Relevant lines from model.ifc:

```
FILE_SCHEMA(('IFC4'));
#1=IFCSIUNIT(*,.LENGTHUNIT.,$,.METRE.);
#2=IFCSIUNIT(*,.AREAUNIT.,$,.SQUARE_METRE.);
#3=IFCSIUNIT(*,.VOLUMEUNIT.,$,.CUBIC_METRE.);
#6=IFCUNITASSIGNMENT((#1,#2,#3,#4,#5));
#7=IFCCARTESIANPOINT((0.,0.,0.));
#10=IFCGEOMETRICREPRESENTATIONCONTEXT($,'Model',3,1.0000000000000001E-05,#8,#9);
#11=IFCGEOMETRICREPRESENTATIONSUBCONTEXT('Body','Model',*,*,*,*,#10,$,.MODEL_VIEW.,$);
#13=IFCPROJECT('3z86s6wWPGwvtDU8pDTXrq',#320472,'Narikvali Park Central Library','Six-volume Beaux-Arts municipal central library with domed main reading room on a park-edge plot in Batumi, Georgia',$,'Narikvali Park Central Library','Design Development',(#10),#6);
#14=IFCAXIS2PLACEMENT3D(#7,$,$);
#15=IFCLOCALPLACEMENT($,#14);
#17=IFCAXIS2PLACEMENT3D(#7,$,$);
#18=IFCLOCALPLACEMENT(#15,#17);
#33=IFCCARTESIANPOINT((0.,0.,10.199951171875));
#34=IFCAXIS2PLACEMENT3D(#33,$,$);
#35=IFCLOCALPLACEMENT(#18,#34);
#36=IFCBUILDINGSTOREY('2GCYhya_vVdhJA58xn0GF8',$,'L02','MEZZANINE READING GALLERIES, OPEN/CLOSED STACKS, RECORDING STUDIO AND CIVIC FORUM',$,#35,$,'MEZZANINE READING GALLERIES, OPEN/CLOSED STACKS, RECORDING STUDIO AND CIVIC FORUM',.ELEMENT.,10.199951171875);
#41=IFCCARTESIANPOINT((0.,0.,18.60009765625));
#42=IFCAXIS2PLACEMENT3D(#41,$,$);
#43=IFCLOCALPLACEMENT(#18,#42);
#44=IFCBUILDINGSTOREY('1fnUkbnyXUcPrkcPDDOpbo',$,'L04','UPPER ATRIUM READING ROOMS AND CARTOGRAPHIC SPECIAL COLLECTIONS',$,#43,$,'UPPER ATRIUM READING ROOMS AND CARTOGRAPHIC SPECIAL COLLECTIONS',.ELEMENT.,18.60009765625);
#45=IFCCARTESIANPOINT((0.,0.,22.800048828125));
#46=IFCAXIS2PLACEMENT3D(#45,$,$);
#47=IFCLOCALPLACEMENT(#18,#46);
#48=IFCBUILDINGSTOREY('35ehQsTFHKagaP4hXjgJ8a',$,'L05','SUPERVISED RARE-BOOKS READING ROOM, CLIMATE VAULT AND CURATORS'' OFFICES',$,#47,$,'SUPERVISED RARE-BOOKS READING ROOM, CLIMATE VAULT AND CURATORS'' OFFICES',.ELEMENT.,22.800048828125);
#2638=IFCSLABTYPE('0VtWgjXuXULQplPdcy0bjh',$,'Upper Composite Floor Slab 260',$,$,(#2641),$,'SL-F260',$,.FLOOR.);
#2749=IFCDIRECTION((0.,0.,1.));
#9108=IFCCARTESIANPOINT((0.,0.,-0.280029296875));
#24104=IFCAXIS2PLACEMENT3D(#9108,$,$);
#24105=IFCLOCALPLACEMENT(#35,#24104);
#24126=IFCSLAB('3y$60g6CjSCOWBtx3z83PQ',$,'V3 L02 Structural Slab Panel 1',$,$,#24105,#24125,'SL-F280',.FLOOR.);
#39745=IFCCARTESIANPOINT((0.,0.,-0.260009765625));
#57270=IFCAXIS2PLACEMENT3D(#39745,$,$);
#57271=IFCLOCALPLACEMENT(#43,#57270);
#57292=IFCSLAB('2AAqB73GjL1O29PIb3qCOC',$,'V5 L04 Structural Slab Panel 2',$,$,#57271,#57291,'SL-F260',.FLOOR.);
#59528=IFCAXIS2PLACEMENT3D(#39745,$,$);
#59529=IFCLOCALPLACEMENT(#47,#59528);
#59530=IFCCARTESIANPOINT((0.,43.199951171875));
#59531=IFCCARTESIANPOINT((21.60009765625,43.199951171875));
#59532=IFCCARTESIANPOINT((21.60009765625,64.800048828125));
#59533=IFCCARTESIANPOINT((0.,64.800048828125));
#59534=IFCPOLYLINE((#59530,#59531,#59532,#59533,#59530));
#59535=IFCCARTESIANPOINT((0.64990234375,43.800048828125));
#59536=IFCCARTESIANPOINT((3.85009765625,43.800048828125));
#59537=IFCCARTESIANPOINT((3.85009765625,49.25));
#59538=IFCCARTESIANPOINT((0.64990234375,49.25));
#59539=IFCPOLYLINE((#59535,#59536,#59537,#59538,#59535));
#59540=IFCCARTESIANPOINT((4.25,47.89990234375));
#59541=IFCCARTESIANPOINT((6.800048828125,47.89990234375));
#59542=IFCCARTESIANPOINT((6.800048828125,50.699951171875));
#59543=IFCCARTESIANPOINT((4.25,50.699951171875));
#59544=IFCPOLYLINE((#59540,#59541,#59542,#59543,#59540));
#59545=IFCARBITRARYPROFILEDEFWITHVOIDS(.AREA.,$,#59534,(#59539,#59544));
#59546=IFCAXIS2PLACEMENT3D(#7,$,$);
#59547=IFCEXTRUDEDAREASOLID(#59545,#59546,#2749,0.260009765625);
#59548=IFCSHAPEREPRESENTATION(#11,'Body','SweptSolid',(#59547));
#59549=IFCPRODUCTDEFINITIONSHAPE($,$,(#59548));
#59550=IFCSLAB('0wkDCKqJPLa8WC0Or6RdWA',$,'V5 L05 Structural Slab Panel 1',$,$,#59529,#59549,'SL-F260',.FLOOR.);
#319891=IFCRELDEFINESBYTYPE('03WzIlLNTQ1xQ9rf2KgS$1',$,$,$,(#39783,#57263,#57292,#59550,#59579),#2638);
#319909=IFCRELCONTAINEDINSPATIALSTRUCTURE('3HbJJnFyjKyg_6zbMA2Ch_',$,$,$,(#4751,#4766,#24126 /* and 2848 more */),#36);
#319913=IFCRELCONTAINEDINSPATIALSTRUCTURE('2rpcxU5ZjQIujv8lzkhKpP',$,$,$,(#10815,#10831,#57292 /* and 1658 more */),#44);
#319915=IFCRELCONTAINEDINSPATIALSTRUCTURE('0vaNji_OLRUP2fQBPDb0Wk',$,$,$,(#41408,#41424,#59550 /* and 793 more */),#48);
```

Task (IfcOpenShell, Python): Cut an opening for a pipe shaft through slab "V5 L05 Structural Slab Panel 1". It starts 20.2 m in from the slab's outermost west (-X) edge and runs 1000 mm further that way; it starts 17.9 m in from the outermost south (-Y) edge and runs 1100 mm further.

```python
import numpy as np
import ifcopenshell
import ifcopenshell.api.feature
import ifcopenshell.api.geometry
import ifcopenshell.api.root
import ifcopenshell.geom
import ifcopenshell.util.placement
import ifcopenshell.util.representation
import ifcopenshell.util.shape
import ifcopenshell.util.unit

model = ifcopenshell.open("model.ifc")
unit_scale = ifcopenshell.util.unit.calculate_unit_scale(model)
settings = ifcopenshell.geom.settings()


def volume(element):
    """Net volume in cubic metres, openings subtracted."""
    shape = ifcopenshell.geom.create_shape(settings, element)
    return ifcopenshell.util.shape.get_volume(shape.geometry)


slab = model.by_guid("0wkDCKqJPLa8WC0Or6RdWA")
before = volume(slab)

# Extent in the slab's own axes, in metres. The edges named are its -X and -Y sides.
slab_shape = ifcopenshell.geom.create_shape(settings, slab)
vertices = ifcopenshell.util.shape.get_vertices(slab_shape.geometry)
x_min, y_min, bottom = vertices.min(axis=0)
top = vertices[:, 2].max()

opening = ifcopenshell.api.root.create_entity(model, ifc_class="IfcOpeningElement", name="Pipe shaft opening", predefined_type="OPENING")
context = ifcopenshell.util.representation.get_context(model, "Model", "Body", "MODEL_VIEW")
width, depth = 1, 1.1
outline = [(0.0, 0.0), (width, 0.0), (width, depth), (0.0, depth), (0.0, 0.0)]
# Overshoot both faces by 50 mm so the cut is clean.
shape = ifcopenshell.api.geometry.add_slab_representation(
    model, context=context, depth=top - bottom + 0.1, polyline=outline
)
ifcopenshell.api.geometry.assign_representation(model, product=opening, representation=shape)

matrix = ifcopenshell.util.placement.get_local_placement(slab.ObjectPlacement)
matrix[:, 3] = matrix @ np.append(np.array([x_min + 20.2, y_min + 17.9, bottom - 0.05]) / unit_scale, 1.0)
ifcopenshell.api.geometry.edit_object_placement(model, product=opening, matrix=matrix, is_si=False)
ifcopenshell.api.feature.add_feature(model, feature=opening, element=slab)

after = volume(slab)

print(f"slab volume {before:.3f} -> {after:.3f} m3")

model.write("model_edited.ifc")
```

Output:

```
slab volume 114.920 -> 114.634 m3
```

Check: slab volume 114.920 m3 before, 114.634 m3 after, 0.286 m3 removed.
